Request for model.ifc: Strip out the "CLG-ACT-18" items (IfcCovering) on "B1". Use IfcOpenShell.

First a look at what the model holds.

```python
import ifcopenshell
import ifcopenshell.util.element

model = ifcopenshell.open("model.ifc")
print(model.schema)
storey = next(s for s in model.by_type("IfcBuildingStorey") if s.Name == "B1")
coverings = [e for e in ifcopenshell.util.element.get_decomposition(storey) if e.is_a("IfcCovering")]
seen = {}
for e in coverings:
    element_type = ifcopenshell.util.element.get_type(e)
    name = element_type.Name if element_type not in (None, e) else None
    seen[name] = seen.get(name, 0) + 1
for name, count in sorted(seen.items(), key=str):
    print(count, "x", name)
```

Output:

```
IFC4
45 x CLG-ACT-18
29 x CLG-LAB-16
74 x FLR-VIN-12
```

```python
import ifcopenshell
import ifcopenshell.api.root
import ifcopenshell.util.element

model = ifcopenshell.open("model.ifc")

storey = next(s for s in model.by_type("IfcBuildingStorey") if s.Name == "B1")
coverings = [e for e in ifcopenshell.util.element.get_decomposition(storey) if e.is_a("IfcCovering")]
targets = [e for e in coverings if (t := ifcopenshell.util.element.get_type(e)) not in (None, e) and t.Name == "CLG-ACT-18"]

for e in targets:
    ifcopenshell.api.root.remove_product(model, product=e)
print(len(targets), "removed")

model.write("model_edited.ifc")
```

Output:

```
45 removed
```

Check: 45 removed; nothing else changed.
